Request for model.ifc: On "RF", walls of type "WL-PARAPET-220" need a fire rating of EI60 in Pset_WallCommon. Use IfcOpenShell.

First a look at what the model holds.

```python
import ifcopenshell
import ifcopenshell.util.element

model = ifcopenshell.open("model.ifc")
print(model.schema)
storey = next(s for s in model.by_type("IfcBuildingStorey") if s.Name == "RF")
walls = [e for e in ifcopenshell.util.element.get_decomposition(storey) if e.is_a("IfcWall")]
seen = {}
for e in walls:
    element_type = ifcopenshell.util.element.get_type(e)
    key = (element_type.Name if element_type != e and element_type else None, ifcopenshell.util.element.get_pset(e, "Pset_WallCommon", "FireRating"))
    seen[key] = seen.get(key, 0) + 1
for (name, value), count in sorted(seen.items(), key=str):
    print(count, "x", name, "|", value)
```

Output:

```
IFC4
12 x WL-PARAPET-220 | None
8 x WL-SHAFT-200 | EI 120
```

```python
import ifcopenshell
import ifcopenshell.api.pset
import ifcopenshell.util.element

model = ifcopenshell.open("model.ifc")

storey = next(s for s in model.by_type("IfcBuildingStorey") if s.Name == "RF")
walls = [e for e in ifcopenshell.util.element.get_decomposition(storey) if e.is_a("IfcWall")]

count = 0
for e in walls:
    element_type = ifcopenshell.util.element.get_type(e)
    if element_type in (None, e) or element_type.Name != "WL-PARAPET-220":
        continue
    # add_pset returns the element's existing set when there is one.
    pset = ifcopenshell.api.pset.add_pset(model, product=e, name="Pset_WallCommon")
    ifcopenshell.api.pset.edit_pset(model, pset=pset, properties={"FireRating": "EI60"})
    count += 1

print(count, "walls updated")

model.write("model_updated.ifc")
```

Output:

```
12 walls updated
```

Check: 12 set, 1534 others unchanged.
